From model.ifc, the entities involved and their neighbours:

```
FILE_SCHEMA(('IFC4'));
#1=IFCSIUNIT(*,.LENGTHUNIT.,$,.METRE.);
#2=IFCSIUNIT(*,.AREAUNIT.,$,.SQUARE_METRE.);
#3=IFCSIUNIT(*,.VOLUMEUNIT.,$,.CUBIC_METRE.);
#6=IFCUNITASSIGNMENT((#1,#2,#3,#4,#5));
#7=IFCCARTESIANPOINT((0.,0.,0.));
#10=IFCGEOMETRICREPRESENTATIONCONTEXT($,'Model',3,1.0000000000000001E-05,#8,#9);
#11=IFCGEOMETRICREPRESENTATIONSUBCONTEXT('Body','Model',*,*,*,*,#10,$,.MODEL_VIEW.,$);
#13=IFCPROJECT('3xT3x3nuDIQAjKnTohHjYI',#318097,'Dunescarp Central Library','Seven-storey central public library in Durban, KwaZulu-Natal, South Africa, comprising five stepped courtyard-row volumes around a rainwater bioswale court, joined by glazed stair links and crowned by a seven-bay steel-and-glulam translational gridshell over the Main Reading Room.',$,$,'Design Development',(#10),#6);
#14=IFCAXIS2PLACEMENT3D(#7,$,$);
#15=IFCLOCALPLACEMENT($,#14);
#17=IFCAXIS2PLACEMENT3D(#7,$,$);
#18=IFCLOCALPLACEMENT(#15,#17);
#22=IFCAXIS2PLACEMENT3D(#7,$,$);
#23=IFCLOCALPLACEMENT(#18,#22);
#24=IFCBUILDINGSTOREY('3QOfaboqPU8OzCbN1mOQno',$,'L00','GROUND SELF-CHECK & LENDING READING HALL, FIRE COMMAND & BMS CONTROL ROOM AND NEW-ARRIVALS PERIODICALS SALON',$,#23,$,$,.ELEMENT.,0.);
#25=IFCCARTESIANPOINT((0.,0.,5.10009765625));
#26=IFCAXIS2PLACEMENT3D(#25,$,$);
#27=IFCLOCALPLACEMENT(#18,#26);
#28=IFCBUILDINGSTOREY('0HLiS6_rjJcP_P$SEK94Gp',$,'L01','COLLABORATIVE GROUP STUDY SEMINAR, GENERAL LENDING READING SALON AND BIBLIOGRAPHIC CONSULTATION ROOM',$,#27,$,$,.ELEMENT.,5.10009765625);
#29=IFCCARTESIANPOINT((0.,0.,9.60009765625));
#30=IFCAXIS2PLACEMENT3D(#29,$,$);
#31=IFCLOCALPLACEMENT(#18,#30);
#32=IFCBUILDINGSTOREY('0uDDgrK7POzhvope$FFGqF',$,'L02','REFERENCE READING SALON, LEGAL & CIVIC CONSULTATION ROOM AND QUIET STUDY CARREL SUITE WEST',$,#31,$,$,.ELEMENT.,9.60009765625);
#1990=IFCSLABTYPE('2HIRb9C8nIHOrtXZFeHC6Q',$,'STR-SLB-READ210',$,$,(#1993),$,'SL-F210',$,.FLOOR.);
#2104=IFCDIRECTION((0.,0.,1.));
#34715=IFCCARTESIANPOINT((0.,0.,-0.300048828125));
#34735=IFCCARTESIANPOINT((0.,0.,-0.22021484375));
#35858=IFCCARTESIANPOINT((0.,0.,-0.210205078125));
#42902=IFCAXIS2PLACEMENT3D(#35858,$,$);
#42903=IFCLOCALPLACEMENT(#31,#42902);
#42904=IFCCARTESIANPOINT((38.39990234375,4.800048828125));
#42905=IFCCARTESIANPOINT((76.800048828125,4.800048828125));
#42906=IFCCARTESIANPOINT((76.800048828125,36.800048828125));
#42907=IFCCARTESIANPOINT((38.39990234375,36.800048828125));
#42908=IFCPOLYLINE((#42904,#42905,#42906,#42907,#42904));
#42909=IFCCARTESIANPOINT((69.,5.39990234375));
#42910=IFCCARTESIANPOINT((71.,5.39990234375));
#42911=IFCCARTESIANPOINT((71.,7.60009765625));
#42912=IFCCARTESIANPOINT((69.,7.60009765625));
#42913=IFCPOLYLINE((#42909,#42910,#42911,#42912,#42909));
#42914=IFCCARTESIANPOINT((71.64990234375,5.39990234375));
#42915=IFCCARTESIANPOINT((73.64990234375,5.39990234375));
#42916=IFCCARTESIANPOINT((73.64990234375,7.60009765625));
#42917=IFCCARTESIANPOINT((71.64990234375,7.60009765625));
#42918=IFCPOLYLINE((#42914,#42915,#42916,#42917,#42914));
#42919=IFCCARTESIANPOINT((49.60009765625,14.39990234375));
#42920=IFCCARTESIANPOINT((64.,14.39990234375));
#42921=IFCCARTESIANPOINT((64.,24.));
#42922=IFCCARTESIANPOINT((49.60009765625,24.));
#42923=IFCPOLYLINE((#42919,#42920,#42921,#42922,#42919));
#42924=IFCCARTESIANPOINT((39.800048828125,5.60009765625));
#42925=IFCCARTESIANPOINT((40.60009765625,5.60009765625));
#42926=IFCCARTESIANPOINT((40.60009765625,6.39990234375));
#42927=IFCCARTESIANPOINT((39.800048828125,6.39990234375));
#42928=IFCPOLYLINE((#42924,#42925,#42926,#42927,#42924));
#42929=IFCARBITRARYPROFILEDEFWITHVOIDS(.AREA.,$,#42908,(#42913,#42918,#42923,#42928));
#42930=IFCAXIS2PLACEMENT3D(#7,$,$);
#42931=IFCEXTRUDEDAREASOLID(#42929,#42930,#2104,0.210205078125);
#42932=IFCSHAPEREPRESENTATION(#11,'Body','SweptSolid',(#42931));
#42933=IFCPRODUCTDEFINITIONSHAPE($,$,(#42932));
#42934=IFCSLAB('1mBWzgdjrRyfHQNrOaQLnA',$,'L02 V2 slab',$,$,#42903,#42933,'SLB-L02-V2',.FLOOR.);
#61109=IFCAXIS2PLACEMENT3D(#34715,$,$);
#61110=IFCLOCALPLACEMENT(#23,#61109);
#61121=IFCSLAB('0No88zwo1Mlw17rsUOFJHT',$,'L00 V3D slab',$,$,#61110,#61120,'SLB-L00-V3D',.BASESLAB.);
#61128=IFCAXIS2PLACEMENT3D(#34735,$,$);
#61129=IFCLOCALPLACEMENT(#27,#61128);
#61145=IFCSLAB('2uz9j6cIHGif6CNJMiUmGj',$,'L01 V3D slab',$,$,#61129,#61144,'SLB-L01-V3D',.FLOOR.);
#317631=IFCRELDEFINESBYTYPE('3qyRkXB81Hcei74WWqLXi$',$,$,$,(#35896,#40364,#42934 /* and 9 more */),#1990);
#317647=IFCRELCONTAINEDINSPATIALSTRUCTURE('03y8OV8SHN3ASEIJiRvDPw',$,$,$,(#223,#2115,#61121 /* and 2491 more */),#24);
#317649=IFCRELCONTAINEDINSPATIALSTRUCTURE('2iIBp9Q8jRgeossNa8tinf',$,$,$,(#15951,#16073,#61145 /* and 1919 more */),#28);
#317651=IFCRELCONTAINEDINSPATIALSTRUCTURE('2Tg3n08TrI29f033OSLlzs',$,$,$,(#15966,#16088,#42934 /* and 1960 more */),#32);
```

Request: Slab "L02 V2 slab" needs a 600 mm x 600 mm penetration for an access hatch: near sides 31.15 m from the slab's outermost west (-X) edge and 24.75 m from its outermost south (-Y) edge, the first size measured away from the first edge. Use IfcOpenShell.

```python
import numpy as np
import ifcopenshell
import ifcopenshell.api.feature
import ifcopenshell.api.geometry
import ifcopenshell.api.root
import ifcopenshell.geom
import ifcopenshell.util.placement
import ifcopenshell.util.representation
import ifcopenshell.util.shape
import ifcopenshell.util.unit

model = ifcopenshell.open("model.ifc")
unit_scale = ifcopenshell.util.unit.calculate_unit_scale(model)
settings = ifcopenshell.geom.settings()


def volume(element):
    """Net volume in cubic metres, openings subtracted."""
    shape = ifcopenshell.geom.create_shape(settings, element)
    return ifcopenshell.util.shape.get_volume(shape.geometry)


slab = model.by_guid("1mBWzgdjrRyfHQNrOaQLnA")
before = volume(slab)

# Extent in the slab's own axes, in metres. The edges named are its -X and -Y sides.
slab_shape = ifcopenshell.geom.create_shape(settings, slab)
vertices = ifcopenshell.util.shape.get_vertices(slab_shape.geometry)
x_min, y_min, bottom = vertices.min(axis=0)
top = vertices[:, 2].max()

opening = ifcopenshell.api.root.create_entity(model, ifc_class="IfcOpeningElement", name="Access hatch opening", predefined_type="OPENING")
context = ifcopenshell.util.representation.get_context(model, "Model", "Body", "MODEL_VIEW")
width, depth = 0.6, 0.6
outline = [(0.0, 0.0), (width, 0.0), (width, depth), (0.0, depth), (0.0, 0.0)]
# Overshoot both faces by 50 mm so the cut is clean.
shape = ifcopenshell.api.geometry.add_slab_representation(
    model, context=context, depth=top - bottom + 0.1, polyline=outline
)
ifcopenshell.api.geometry.assign_representation(model, product=opening, representation=shape)

matrix = ifcopenshell.util.placement.get_local_placement(slab.ObjectPlacement)
matrix[:, 3] = matrix @ np.append(np.array([x_min + 31.15, y_min + 24.75, bottom - 0.05]) / unit_scale, 1.0)
ifcopenshell.api.geometry.edit_object_placement(model, product=opening, matrix=matrix, is_si=False)
ifcopenshell.api.feature.add_feature(model, feature=opening, element=slab)

after = volume(slab)

print(f"slab volume {before:.3f} -> {after:.3f} m3")

model.write("model-out.ifc")
```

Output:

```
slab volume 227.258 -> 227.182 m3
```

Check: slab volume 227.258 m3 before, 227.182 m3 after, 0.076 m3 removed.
